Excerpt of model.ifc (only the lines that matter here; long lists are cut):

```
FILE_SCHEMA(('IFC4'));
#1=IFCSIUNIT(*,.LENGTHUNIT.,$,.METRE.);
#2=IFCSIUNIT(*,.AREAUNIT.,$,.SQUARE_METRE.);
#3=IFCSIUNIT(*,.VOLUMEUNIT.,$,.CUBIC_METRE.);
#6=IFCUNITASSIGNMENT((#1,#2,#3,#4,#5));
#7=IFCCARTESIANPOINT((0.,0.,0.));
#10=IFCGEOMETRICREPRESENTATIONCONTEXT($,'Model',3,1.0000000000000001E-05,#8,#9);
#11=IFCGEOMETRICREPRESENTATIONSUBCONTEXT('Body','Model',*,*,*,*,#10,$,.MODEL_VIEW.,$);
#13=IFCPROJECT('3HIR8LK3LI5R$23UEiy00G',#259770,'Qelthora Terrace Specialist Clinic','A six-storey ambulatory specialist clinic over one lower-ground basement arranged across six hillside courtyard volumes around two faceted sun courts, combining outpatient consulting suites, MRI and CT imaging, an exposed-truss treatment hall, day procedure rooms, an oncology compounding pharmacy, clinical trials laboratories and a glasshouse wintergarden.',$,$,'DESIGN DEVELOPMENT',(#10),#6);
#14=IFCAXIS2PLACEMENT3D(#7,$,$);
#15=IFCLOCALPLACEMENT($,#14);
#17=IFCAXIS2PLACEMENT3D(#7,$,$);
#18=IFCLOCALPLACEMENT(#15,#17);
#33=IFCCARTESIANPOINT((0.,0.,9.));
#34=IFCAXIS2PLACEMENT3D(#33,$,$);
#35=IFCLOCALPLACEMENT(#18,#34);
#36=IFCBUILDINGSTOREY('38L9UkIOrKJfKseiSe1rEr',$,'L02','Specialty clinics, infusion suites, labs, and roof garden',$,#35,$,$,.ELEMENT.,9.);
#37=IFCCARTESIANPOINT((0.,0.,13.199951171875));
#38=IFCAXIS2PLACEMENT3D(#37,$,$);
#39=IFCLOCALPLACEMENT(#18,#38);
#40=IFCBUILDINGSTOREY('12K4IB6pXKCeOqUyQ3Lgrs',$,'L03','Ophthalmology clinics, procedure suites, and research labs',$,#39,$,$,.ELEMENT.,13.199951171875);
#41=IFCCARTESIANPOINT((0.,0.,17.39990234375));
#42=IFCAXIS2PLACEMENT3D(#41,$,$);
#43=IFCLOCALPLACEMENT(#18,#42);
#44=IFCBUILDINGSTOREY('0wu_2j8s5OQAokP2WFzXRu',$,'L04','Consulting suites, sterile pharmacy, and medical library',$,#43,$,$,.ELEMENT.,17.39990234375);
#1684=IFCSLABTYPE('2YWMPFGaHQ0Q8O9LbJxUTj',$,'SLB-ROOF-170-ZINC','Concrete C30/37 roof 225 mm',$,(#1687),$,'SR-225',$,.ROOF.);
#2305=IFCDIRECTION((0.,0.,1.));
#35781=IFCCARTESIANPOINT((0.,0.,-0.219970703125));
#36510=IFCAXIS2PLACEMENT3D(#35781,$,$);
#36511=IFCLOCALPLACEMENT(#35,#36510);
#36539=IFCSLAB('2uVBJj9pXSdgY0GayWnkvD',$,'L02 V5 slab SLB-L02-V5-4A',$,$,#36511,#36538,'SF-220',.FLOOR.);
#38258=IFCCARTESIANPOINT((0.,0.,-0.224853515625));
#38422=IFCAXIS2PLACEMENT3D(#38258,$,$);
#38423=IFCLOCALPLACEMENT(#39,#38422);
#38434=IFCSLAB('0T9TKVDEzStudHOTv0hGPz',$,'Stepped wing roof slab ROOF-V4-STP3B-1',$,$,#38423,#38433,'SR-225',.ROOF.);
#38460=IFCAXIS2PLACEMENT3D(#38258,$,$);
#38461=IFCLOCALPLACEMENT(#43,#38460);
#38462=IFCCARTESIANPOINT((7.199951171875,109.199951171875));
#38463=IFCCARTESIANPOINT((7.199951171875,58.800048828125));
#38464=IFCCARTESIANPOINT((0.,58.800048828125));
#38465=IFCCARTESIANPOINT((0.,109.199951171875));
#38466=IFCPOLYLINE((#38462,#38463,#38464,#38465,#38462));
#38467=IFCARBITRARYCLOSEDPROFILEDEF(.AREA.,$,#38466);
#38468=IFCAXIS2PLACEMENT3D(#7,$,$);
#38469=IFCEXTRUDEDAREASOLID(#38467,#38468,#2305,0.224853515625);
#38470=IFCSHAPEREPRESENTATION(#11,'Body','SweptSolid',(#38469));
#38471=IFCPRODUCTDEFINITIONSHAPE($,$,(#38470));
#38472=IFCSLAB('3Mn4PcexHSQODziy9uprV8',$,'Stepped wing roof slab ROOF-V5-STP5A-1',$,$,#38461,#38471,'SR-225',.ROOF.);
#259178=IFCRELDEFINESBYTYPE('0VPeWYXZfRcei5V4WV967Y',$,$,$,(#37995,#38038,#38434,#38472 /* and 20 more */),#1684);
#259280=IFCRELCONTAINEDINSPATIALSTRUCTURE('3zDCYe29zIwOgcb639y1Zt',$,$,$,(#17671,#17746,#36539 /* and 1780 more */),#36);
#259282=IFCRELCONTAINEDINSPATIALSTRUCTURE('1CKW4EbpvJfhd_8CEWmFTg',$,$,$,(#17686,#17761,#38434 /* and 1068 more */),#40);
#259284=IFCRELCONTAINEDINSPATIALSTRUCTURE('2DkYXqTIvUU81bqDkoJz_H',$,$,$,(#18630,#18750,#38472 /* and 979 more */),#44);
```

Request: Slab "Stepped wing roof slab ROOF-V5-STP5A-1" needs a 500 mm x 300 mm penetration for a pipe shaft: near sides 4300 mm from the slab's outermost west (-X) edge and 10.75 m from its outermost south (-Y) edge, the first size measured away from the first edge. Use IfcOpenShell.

```python
import numpy as np
import ifcopenshell
import ifcopenshell.api.feature
import ifcopenshell.api.geometry
import ifcopenshell.api.root
import ifcopenshell.geom
import ifcopenshell.util.placement
import ifcopenshell.util.representation
import ifcopenshell.util.shape
import ifcopenshell.util.unit

model = ifcopenshell.open("model.ifc")
unit_scale = ifcopenshell.util.unit.calculate_unit_scale(model)
settings = ifcopenshell.geom.settings()


def volume(element):
    """Net volume in cubic metres, openings subtracted."""
    shape = ifcopenshell.geom.create_shape(settings, element)
    return ifcopenshell.util.shape.get_volume(shape.geometry)


slab = model.by_guid("3Mn4PcexHSQODziy9uprV8")
before = volume(slab)

# Extent in the slab's own axes, in metres. The edges named are its -X and -Y sides.
slab_shape = ifcopenshell.geom.create_shape(settings, slab)
vertices = ifcopenshell.util.shape.get_vertices(slab_shape.geometry)
x_min, y_min, bottom = vertices.min(axis=0)
top = vertices[:, 2].max()

opening = ifcopenshell.api.root.create_entity(model, ifc_class="IfcOpeningElement", name="Pipe shaft opening", predefined_type="OPENING")
context = ifcopenshell.util.representation.get_context(model, "Model", "Body", "MODEL_VIEW")
width, depth = 0.5, 0.3
outline = [(0.0, 0.0), (width, 0.0), (width, depth), (0.0, depth), (0.0, 0.0)]
# Overshoot both faces by 50 mm so the cut is clean.
shape = ifcopenshell.api.geometry.add_slab_representation(
    model, context=context, depth=top - bottom + 0.1, polyline=outline
)
ifcopenshell.api.geometry.assign_representation(model, product=opening, representation=shape)

matrix = ifcopenshell.util.placement.get_local_placement(slab.ObjectPlacement)
matrix[:, 3] = matrix @ np.append(np.array([x_min + 4.3, y_min + 10.75, bottom - 0.05]) / unit_scale, 1.0)
ifcopenshell.api.geometry.edit_object_placement(model, product=opening, matrix=matrix, is_si=False)
ifcopenshell.api.feature.add_feature(model, feature=opening, element=slab)

after = volume(slab)

print(f"slab volume {before:.3f} -> {after:.3f} m3")

model.write("model_edited.ifc")
```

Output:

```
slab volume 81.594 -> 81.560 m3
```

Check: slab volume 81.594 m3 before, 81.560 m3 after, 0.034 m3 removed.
